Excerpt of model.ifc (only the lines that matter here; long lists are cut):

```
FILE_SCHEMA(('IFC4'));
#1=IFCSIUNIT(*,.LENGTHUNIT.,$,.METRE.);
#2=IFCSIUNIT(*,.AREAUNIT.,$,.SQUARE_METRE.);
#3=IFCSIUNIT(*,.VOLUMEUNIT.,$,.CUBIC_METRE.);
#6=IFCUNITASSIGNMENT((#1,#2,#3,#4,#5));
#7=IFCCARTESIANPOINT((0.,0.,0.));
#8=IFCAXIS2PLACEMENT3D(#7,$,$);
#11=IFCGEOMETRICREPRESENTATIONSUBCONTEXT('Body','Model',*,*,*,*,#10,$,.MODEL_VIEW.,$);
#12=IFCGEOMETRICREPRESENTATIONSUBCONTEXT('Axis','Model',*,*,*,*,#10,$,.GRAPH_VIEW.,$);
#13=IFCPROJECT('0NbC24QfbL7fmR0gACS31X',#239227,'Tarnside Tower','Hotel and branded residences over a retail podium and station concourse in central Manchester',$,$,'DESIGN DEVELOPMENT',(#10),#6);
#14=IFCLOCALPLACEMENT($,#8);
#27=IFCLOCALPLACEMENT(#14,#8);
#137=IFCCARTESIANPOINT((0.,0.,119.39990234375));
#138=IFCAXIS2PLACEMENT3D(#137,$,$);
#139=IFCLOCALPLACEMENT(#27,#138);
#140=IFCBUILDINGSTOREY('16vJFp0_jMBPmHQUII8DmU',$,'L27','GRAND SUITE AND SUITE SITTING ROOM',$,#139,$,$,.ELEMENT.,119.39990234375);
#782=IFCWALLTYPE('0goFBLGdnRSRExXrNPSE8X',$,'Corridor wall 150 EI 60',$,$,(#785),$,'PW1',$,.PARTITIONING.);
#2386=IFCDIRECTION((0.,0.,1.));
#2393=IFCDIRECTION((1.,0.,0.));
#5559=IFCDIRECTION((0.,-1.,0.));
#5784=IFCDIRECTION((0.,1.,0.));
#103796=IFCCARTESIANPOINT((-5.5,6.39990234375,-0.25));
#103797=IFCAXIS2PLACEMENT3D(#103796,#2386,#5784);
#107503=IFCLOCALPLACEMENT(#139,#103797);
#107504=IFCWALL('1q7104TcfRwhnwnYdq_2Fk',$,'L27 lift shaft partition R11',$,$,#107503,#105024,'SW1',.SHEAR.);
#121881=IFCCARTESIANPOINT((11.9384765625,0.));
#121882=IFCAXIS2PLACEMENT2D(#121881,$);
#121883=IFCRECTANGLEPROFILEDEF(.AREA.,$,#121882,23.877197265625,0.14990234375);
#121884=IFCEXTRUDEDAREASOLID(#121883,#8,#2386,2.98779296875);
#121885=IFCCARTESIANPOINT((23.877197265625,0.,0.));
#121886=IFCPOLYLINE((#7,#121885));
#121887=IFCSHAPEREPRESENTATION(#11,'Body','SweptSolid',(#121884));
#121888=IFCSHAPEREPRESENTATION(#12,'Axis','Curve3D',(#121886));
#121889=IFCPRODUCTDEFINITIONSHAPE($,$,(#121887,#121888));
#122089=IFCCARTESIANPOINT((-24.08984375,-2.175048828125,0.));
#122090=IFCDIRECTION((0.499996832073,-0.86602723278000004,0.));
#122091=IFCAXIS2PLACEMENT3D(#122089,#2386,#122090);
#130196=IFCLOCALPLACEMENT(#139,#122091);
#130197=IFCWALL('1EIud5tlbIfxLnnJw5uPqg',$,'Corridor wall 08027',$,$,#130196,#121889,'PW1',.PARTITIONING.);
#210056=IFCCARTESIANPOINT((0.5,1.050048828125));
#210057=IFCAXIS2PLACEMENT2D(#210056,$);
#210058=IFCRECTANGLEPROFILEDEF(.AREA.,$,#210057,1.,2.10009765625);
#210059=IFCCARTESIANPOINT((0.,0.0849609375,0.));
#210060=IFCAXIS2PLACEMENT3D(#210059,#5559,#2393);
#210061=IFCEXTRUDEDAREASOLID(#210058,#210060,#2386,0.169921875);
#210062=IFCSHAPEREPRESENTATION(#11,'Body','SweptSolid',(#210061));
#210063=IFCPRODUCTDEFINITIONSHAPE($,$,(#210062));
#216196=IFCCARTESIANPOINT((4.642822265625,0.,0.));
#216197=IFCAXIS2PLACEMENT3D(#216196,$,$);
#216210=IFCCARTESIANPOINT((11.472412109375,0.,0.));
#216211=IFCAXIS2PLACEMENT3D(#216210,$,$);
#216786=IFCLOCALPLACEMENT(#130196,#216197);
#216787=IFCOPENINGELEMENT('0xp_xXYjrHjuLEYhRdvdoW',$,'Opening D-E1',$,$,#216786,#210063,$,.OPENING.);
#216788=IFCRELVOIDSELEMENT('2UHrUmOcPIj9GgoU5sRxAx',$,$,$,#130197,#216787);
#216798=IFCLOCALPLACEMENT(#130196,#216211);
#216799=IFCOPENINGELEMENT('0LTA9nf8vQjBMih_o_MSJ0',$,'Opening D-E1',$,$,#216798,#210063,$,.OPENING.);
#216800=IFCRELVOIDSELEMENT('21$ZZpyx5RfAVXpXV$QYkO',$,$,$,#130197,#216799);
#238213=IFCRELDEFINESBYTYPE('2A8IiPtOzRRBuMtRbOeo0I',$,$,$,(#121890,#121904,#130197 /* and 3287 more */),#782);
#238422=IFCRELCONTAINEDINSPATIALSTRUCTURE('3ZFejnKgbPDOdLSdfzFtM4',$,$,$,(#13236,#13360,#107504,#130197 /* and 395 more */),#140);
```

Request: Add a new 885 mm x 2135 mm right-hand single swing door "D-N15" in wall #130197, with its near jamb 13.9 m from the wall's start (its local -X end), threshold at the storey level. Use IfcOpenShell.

```python
import numpy as np
import ifcopenshell
import ifcopenshell.api.feature
import ifcopenshell.api.geometry
import ifcopenshell.api.root
import ifcopenshell.api.spatial
import ifcopenshell.geom
import ifcopenshell.util.element
import ifcopenshell.util.placement
import ifcopenshell.util.representation
import ifcopenshell.util.shape
import ifcopenshell.util.unit

model = ifcopenshell.open("model.ifc")
unit_scale = ifcopenshell.util.unit.calculate_unit_scale(model)
settings = ifcopenshell.geom.settings()


def volume(element):
    """Net volume in cubic metres, openings subtracted."""
    shape = ifcopenshell.geom.create_shape(settings, element)
    return ifcopenshell.util.shape.get_volume(shape.geometry)


wall = model.by_guid("1EIud5tlbIfxLnnJw5uPqg")
storey = ifcopenshell.util.element.get_container(wall, ifc_class="IfcBuildingStorey")
context = ifcopenshell.util.representation.get_context(model, "Model", "Body", "MODEL_VIEW")
before = volume(wall)

width, height, from_end, sill = 0.885, 2.135, 13.9, 0.0  # metres

# The wall runs along its own X axis, and the end named is its -X end.
wall_shape = ifcopenshell.geom.create_shape(settings, wall)
x, y, z = ifcopenshell.util.shape.get_vertices(wall_shape.geometry).T
start = x.min() + from_end
face, thickness = float(y.min()), float(y.max() - y.min())
wall_matrix = ifcopenshell.util.placement.get_local_placement(wall.ObjectPlacement)
level = ifcopenshell.util.placement.get_local_placement(storey.ObjectPlacement)[2, 3]


def in_wall(x, y):
    """Placement at x, y metres in the wall's axes, at sill height."""
    matrix = wall_matrix.copy()
    matrix[:, 3] = wall_matrix @ np.array([x / unit_scale, y / unit_scale, 0.0, 1.0])
    matrix[2, 3] = level + sill / unit_scale
    return matrix


# Opening: a box that overshoots both wall faces by 50 mm.
opening = ifcopenshell.api.root.create_entity(model, ifc_class="IfcOpeningElement", predefined_type="OPENING")
box = ifcopenshell.api.geometry.add_wall_representation(
    model, context=context, length=width, height=height, thickness=thickness + 0.1
)
ifcopenshell.api.geometry.assign_representation(model, product=opening, representation=box)
ifcopenshell.api.geometry.edit_object_placement(model, product=opening, matrix=in_wall(start, face - 0.05), is_si=False)
ifcopenshell.api.feature.add_feature(model, feature=opening, element=wall)

door = ifcopenshell.api.root.create_entity(model, ifc_class="IfcDoor", name="D-N15", predefined_type="DOOR")
door.OverallWidth, door.OverallHeight = width / unit_scale, height / unit_scale
door.OperationType = "SINGLE_SWING_RIGHT"
body = ifcopenshell.api.geometry.add_door_representation(
    model,
    context=context,
    overall_width=door.OverallWidth,
    overall_height=door.OverallHeight,
    operation_type="SINGLE_SWING_RIGHT",
    lining_properties={"LiningDepth": thickness / unit_scale, "ThresholdDepth": thickness / unit_scale},
)
ifcopenshell.api.geometry.assign_representation(model, product=door, representation=body)
ifcopenshell.api.spatial.assign_container(model, products=[door], relating_structure=storey)
ifcopenshell.api.feature.add_filling(model, opening=opening, element=door)

# The lining spans the wall, so the door starts at the wall face.
ifcopenshell.api.geometry.edit_object_placement(model, product=door, matrix=in_wall(start, face), is_si=False)

after = volume(wall)

print(f"wall volume {before:.3f} -> {after:.3f} m3")

model.write("model_updated.ifc")
```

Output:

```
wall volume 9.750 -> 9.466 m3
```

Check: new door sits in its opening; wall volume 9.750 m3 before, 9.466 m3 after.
